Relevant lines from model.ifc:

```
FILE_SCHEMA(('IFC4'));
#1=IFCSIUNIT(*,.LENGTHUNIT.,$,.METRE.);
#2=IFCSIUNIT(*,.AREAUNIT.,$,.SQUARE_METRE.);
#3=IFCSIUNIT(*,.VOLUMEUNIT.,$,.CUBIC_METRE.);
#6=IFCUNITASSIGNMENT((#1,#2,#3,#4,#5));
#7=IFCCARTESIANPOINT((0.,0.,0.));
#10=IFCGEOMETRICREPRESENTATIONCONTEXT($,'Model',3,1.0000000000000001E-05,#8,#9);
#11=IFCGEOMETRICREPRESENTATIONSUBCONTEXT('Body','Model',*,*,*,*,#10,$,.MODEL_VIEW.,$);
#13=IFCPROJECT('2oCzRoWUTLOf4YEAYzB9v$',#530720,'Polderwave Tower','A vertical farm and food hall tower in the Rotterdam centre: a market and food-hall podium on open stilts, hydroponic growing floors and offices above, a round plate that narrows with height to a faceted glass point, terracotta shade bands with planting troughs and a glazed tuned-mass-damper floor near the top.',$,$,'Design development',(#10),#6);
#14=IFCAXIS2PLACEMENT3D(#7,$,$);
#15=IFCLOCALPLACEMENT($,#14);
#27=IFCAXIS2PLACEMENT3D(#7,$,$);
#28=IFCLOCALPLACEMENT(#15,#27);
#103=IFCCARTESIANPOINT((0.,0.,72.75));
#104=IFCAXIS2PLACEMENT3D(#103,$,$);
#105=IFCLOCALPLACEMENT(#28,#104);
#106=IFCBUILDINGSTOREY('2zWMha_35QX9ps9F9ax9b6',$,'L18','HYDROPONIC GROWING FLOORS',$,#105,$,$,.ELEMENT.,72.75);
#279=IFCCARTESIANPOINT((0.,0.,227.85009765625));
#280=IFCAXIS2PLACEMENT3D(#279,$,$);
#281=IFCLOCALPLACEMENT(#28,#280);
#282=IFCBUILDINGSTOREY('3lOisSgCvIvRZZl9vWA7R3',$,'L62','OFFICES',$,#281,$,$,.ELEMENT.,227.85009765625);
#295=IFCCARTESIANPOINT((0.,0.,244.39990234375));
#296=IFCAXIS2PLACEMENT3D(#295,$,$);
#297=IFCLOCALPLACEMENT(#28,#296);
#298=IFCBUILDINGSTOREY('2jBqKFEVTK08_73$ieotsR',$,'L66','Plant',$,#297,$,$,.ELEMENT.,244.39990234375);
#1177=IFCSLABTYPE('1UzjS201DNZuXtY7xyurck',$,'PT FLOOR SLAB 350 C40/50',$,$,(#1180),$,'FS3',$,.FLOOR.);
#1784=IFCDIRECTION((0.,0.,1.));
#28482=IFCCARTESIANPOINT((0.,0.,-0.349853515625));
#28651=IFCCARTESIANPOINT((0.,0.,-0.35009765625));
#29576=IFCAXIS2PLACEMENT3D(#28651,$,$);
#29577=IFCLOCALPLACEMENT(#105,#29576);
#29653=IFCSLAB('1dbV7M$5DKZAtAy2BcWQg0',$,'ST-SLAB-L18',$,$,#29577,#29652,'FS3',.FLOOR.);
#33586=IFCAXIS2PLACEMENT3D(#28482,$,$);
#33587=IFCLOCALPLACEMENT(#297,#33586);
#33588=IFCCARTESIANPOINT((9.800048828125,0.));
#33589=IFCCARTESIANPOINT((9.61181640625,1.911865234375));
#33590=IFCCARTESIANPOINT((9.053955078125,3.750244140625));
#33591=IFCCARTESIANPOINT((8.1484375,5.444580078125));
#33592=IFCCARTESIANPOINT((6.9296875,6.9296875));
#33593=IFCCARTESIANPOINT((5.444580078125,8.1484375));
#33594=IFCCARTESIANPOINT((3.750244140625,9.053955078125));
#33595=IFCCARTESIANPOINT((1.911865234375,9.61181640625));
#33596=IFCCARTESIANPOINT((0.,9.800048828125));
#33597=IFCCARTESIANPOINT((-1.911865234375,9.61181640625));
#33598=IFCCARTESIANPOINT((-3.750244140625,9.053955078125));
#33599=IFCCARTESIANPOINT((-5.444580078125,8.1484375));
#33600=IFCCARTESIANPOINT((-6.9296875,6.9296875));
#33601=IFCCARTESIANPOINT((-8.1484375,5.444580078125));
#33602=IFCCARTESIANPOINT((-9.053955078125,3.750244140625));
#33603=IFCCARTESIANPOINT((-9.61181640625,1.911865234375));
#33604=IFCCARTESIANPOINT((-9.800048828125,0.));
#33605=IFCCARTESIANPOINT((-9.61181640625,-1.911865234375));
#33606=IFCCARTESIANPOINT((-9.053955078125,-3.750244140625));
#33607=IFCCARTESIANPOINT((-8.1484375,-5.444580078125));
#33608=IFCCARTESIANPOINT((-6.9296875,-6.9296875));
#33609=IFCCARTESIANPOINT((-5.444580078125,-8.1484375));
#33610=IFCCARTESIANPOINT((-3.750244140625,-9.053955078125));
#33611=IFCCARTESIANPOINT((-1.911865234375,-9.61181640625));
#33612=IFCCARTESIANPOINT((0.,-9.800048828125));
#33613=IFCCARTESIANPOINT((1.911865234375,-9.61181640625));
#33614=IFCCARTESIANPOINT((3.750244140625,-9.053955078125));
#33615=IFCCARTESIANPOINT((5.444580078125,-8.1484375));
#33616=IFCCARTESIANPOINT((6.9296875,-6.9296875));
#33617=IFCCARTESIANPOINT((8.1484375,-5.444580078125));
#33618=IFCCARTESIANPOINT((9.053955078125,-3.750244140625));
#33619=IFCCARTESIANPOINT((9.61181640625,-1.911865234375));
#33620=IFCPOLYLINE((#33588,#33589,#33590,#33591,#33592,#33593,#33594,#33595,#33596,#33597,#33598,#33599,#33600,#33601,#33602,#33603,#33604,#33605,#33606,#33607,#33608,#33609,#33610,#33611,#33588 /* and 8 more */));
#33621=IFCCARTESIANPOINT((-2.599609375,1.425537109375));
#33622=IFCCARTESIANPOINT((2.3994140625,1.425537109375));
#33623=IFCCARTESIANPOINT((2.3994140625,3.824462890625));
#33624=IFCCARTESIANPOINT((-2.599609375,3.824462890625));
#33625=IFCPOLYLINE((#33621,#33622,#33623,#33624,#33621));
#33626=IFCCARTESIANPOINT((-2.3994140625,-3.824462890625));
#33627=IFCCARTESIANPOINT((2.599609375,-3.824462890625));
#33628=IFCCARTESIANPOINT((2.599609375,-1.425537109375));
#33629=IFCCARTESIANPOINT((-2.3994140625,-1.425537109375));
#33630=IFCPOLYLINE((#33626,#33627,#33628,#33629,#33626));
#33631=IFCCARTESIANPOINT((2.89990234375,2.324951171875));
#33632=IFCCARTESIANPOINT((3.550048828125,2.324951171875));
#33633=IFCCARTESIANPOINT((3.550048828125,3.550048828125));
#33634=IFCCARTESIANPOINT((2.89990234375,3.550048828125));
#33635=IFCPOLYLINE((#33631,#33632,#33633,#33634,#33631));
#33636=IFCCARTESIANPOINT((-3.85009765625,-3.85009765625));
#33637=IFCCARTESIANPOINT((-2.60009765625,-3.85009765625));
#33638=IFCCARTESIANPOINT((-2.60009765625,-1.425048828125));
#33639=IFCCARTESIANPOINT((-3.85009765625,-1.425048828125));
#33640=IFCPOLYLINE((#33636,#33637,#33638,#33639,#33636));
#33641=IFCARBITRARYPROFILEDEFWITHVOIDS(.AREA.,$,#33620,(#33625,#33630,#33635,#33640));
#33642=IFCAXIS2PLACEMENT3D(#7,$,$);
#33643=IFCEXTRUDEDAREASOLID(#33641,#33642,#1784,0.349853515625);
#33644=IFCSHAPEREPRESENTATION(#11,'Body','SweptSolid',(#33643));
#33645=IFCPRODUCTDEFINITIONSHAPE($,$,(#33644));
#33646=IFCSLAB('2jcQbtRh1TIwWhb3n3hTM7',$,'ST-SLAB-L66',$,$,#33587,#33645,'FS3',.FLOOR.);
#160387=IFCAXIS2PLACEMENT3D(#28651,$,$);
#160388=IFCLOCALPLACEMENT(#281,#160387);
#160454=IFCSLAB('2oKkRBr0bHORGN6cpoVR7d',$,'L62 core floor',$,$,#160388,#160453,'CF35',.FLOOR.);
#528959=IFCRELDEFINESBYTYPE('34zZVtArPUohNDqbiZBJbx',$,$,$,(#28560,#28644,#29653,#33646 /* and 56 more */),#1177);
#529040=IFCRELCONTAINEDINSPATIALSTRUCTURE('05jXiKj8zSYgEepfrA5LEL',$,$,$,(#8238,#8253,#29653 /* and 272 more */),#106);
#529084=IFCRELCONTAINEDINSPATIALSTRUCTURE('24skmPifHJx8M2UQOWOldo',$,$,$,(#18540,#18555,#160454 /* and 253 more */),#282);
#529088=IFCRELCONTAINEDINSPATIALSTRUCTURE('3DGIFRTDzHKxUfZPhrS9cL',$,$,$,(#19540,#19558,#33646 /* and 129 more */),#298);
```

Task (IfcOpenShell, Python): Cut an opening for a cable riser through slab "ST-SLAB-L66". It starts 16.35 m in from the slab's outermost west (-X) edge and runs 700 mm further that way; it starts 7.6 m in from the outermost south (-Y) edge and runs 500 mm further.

```python
import numpy as np
import ifcopenshell
import ifcopenshell.api.feature
import ifcopenshell.api.geometry
import ifcopenshell.api.root
import ifcopenshell.geom
import ifcopenshell.util.placement
import ifcopenshell.util.representation
import ifcopenshell.util.shape
import ifcopenshell.util.unit

model = ifcopenshell.open("model.ifc")
unit_scale = ifcopenshell.util.unit.calculate_unit_scale(model)
settings = ifcopenshell.geom.settings()


def volume(element):
    """Net volume in cubic metres, openings subtracted."""
    shape = ifcopenshell.geom.create_shape(settings, element)
    return ifcopenshell.util.shape.get_volume(shape.geometry)


slab = model.by_id(33646)
before = volume(slab)

# Extent in the slab's own axes, in metres. The edges named are its -X and -Y sides.
slab_shape = ifcopenshell.geom.create_shape(settings, slab)
vertices = ifcopenshell.util.shape.get_vertices(slab_shape.geometry)
x_min, y_min, bottom = vertices.min(axis=0)
top = vertices[:, 2].max()

opening = ifcopenshell.api.root.create_entity(model, ifc_class="IfcOpeningElement", name="Cable riser opening", predefined_type="OPENING")
context = ifcopenshell.util.representation.get_context(model, "Model", "Body", "MODEL_VIEW")
width, depth = 0.7, 0.5
outline = [(0.0, 0.0), (width, 0.0), (width, depth), (0.0, depth), (0.0, 0.0)]
# Overshoot both faces by 50 mm so the cut is clean.
shape = ifcopenshell.api.geometry.add_slab_representation(
    model, context=context, depth=top - bottom + 0.1, polyline=outline
)
ifcopenshell.api.geometry.assign_representation(model, product=opening, representation=shape)

matrix = ifcopenshell.util.placement.get_local_placement(slab.ObjectPlacement)
matrix[:, 3] = matrix @ np.append(np.array([x_min + 16.35, y_min + 7.6, bottom - 0.05]) / unit_scale, 1.0)
ifcopenshell.api.geometry.edit_object_placement(model, product=opening, matrix=matrix, is_si=False)
ifcopenshell.api.feature.add_feature(model, feature=opening, element=slab)

after = volume(slab)

print(f"slab volume {before:.3f} -> {after:.3f} m3")

model.write("model_v2.ifc")
```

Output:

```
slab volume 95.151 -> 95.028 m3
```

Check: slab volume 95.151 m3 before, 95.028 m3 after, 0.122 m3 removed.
